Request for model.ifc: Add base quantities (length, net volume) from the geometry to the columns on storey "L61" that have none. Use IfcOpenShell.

First a look at what the model holds.

```python
import ifcopenshell
import ifcopenshell.util.element
import ifcopenshell.util.unit

model = ifcopenshell.open("model.ifc")
print(model.schema)
for unit_type in ("LENGTHUNIT", "AREAUNIT", "VOLUMEUNIT"):
    print(unit_type, ifcopenshell.util.unit.calculate_unit_scale(model, unit_type))
storey = next(s for s in model.by_type("IfcBuildingStorey") if s.Name == "L61")
columns = [e for e in ifcopenshell.util.element.get_decomposition(storey) if e.is_a("IfcColumn")]
for e in sorted(columns, key=lambda e: e.id()):
    print(e.id(), e.is_a(), e.Name, list(ifcopenshell.util.element.get_psets(e, qtos_only=True)), sep=" | ")
```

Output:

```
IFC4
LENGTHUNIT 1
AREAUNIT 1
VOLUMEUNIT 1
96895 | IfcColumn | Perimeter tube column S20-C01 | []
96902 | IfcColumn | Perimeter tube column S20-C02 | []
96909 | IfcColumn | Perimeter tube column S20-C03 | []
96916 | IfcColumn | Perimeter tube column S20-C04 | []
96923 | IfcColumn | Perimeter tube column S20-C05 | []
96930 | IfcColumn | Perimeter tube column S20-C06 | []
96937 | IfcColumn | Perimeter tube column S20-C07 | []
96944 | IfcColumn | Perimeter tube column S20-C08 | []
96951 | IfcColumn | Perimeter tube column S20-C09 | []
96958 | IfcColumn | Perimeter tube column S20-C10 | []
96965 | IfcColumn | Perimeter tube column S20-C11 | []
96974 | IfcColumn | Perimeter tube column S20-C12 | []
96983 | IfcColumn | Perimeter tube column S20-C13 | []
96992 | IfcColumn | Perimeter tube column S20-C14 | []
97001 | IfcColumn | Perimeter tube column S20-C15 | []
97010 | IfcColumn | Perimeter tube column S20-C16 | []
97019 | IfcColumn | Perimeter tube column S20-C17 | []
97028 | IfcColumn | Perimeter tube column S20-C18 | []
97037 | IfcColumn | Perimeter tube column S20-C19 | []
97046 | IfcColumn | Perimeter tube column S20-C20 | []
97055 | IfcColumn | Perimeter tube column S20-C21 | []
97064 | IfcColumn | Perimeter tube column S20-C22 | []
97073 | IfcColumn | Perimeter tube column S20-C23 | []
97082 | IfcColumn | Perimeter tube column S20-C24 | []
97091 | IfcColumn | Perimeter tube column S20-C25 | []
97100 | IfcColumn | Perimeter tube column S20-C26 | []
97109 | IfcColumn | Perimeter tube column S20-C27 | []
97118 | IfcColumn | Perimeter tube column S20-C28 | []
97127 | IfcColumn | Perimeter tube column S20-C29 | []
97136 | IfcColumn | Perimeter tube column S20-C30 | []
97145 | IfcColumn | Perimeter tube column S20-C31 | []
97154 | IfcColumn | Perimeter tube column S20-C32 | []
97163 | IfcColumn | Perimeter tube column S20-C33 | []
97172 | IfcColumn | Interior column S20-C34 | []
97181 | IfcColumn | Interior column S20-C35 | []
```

```python
import ifcopenshell
import ifcopenshell.api.pset
import ifcopenshell.geom
import ifcopenshell.util.element
import ifcopenshell.util.shape
import ifcopenshell.util.unit

model = ifcopenshell.open("model.ifc")
unit_scale = ifcopenshell.util.unit.calculate_unit_scale(model)
volume_scale = ifcopenshell.util.unit.calculate_unit_scale(model, "VOLUMEUNIT")
settings = ifcopenshell.geom.settings()

storey = next(s for s in model.by_type("IfcBuildingStorey") if s.Name == "L61")
columns = [e for e in ifcopenshell.util.element.get_decomposition(storey) if e.is_a("IfcColumn")]

for e in sorted(columns, key=lambda e: e.id()):
    if ifcopenshell.util.element.get_psets(e, qtos_only=True, should_inherit=False):
        continue
    # Geometry comes back in metres, in the element's own axes.
    shape = ifcopenshell.geom.create_shape(settings, e)
    values = {
        "Length": ifcopenshell.util.shape.get_z(shape.geometry) / unit_scale,
        "NetVolume": ifcopenshell.util.shape.get_volume(shape.geometry) / volume_scale,
    }
    qto = ifcopenshell.api.pset.add_qto(model, product=e, name="Qto_ColumnBaseQuantities")
    ifcopenshell.api.pset.edit_qto(model, qto=qto, properties=values)
    print(e.id(), {k: round(v, 3) for k, v in values.items()})

model.write("model_updated.ifc")
```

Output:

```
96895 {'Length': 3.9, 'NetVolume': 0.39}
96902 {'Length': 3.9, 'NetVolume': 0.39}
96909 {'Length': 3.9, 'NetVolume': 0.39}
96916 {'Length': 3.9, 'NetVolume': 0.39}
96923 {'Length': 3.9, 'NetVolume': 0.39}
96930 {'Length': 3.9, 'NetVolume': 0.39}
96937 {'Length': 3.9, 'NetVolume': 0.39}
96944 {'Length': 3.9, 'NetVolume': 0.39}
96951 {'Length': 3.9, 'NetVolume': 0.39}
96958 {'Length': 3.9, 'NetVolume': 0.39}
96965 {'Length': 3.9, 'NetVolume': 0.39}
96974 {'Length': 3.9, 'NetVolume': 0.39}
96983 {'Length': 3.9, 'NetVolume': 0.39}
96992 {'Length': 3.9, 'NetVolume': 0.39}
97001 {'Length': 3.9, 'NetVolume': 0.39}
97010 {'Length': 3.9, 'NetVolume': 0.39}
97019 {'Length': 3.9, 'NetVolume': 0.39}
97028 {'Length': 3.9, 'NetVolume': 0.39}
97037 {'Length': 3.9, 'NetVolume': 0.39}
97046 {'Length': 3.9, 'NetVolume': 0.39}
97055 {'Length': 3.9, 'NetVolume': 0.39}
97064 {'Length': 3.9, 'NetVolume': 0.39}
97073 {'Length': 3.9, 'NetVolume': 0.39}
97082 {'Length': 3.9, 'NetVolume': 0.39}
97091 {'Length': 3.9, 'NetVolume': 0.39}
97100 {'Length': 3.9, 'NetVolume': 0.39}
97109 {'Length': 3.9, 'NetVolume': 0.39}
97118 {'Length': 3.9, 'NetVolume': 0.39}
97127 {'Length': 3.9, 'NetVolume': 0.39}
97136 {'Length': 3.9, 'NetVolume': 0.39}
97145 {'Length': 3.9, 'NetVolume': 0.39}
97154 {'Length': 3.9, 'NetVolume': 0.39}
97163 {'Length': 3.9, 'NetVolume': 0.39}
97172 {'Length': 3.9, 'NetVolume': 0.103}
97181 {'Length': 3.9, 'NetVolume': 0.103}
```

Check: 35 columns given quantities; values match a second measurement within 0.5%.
